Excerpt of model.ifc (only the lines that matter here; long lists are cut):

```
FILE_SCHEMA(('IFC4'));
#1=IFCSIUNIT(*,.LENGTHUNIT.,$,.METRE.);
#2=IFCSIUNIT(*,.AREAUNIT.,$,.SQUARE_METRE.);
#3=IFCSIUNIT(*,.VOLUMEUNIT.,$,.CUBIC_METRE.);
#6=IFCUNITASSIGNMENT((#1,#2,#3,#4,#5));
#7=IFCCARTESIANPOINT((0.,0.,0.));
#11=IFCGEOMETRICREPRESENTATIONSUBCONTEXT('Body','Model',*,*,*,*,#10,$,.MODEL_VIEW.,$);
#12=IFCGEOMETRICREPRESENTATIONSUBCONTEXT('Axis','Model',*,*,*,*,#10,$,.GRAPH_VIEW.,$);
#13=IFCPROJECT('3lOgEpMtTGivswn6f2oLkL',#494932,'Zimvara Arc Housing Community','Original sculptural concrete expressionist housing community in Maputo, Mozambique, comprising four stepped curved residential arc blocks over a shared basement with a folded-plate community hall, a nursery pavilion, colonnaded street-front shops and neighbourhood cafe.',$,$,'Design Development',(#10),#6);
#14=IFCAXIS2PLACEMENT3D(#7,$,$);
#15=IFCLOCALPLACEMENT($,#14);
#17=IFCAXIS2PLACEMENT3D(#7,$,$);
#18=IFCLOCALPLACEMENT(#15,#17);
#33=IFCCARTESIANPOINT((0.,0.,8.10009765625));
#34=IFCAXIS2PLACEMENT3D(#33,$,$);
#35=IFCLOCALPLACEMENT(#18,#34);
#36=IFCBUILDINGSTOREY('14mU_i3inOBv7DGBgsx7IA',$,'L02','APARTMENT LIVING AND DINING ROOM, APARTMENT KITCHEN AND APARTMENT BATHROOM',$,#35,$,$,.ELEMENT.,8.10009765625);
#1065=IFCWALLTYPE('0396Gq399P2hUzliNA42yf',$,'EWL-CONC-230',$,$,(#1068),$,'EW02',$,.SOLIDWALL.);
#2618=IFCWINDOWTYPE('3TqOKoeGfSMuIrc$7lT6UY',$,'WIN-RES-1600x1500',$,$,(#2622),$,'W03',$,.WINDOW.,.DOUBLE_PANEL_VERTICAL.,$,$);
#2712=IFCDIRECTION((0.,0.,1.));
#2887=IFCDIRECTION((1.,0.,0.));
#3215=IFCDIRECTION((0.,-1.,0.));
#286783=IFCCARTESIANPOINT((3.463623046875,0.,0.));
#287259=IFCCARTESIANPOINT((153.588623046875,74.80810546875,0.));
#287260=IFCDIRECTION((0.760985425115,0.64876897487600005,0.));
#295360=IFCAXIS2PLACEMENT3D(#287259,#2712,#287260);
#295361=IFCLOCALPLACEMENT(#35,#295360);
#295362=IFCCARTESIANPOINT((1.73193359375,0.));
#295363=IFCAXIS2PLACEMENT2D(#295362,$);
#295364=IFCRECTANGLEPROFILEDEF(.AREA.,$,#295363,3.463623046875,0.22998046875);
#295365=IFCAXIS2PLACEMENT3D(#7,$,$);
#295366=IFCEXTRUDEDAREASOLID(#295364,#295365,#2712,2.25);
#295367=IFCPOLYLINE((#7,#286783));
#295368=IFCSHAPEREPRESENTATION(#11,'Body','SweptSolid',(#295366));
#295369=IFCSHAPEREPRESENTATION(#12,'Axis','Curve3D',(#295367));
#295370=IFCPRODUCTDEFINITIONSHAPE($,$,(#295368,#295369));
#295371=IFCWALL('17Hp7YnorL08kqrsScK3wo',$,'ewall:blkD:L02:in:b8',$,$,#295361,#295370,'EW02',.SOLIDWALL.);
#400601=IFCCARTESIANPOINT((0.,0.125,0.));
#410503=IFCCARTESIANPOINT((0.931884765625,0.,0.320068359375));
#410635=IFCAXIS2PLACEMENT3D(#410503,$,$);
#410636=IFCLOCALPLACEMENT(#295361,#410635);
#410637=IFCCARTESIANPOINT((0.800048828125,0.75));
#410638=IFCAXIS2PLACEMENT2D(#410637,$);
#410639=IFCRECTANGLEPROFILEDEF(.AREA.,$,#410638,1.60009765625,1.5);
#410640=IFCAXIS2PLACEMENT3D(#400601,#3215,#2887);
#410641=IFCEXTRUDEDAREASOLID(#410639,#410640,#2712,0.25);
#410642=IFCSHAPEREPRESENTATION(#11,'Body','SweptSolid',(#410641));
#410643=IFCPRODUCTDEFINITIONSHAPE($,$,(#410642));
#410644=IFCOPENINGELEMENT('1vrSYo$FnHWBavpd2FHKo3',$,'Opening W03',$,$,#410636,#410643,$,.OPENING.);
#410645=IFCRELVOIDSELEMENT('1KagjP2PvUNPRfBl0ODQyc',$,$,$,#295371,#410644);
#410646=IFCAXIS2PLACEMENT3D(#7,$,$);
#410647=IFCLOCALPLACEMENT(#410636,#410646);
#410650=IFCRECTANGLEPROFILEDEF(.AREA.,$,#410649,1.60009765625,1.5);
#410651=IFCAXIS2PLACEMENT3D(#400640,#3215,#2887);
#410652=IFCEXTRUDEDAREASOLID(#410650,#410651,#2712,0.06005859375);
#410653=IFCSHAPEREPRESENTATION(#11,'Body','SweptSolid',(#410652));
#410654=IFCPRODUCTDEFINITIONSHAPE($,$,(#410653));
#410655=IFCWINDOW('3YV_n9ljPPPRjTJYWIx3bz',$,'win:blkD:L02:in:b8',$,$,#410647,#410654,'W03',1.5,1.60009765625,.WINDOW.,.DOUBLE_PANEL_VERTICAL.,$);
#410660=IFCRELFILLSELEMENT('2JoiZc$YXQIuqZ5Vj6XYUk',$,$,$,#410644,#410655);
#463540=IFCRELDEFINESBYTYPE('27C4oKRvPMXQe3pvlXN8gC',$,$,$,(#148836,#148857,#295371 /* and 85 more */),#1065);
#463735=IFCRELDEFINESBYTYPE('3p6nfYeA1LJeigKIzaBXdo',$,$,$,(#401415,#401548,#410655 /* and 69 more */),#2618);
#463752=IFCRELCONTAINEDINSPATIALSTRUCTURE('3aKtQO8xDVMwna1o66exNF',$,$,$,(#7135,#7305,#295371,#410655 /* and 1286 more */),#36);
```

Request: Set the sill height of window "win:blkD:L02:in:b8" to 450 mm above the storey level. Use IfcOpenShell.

```python
import numpy as np
import ifcopenshell
import ifcopenshell.api.geometry
import ifcopenshell.geom
import ifcopenshell.util.element
import ifcopenshell.util.placement
import ifcopenshell.util.shape
import ifcopenshell.util.unit

model = ifcopenshell.open("model.ifc")
unit_scale = ifcopenshell.util.unit.calculate_unit_scale(model)

window = model.by_guid("3YV_n9ljPPPRjTJYWIx3bz")
opening = window.FillsVoids[0].RelatingOpeningElement
storey = ifcopenshell.util.element.get_container(window, ifc_class="IfcBuildingStorey")
level = ifcopenshell.util.placement.get_local_placement(storey.ObjectPlacement)[2, 3]

# The opening's origin need not be at the sill, so measure its lowest point.
shape = ifcopenshell.geom.create_shape(ifcopenshell.geom.settings(), opening)
bottom = ifcopenshell.util.shape.get_shape_bottom_elevation(shape, shape.geometry) / unit_scale
dz = level + 0.45 / unit_scale - bottom

shift = np.array([0.0, 0.0, dz])
# The window is placed relative to its opening, so it follows when the opening moves.
matrix = ifcopenshell.util.placement.get_local_placement(opening.ObjectPlacement)
matrix[:3, 3] += shift
ifcopenshell.api.geometry.edit_object_placement(
    model, product=opening, matrix=matrix, is_si=False, should_transform_children=True
)

print(f"moved by {dz * unit_scale:+.3f} m")

model.write("model_edited.ifc")
```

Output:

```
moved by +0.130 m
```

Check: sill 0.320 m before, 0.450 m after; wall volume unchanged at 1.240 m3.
